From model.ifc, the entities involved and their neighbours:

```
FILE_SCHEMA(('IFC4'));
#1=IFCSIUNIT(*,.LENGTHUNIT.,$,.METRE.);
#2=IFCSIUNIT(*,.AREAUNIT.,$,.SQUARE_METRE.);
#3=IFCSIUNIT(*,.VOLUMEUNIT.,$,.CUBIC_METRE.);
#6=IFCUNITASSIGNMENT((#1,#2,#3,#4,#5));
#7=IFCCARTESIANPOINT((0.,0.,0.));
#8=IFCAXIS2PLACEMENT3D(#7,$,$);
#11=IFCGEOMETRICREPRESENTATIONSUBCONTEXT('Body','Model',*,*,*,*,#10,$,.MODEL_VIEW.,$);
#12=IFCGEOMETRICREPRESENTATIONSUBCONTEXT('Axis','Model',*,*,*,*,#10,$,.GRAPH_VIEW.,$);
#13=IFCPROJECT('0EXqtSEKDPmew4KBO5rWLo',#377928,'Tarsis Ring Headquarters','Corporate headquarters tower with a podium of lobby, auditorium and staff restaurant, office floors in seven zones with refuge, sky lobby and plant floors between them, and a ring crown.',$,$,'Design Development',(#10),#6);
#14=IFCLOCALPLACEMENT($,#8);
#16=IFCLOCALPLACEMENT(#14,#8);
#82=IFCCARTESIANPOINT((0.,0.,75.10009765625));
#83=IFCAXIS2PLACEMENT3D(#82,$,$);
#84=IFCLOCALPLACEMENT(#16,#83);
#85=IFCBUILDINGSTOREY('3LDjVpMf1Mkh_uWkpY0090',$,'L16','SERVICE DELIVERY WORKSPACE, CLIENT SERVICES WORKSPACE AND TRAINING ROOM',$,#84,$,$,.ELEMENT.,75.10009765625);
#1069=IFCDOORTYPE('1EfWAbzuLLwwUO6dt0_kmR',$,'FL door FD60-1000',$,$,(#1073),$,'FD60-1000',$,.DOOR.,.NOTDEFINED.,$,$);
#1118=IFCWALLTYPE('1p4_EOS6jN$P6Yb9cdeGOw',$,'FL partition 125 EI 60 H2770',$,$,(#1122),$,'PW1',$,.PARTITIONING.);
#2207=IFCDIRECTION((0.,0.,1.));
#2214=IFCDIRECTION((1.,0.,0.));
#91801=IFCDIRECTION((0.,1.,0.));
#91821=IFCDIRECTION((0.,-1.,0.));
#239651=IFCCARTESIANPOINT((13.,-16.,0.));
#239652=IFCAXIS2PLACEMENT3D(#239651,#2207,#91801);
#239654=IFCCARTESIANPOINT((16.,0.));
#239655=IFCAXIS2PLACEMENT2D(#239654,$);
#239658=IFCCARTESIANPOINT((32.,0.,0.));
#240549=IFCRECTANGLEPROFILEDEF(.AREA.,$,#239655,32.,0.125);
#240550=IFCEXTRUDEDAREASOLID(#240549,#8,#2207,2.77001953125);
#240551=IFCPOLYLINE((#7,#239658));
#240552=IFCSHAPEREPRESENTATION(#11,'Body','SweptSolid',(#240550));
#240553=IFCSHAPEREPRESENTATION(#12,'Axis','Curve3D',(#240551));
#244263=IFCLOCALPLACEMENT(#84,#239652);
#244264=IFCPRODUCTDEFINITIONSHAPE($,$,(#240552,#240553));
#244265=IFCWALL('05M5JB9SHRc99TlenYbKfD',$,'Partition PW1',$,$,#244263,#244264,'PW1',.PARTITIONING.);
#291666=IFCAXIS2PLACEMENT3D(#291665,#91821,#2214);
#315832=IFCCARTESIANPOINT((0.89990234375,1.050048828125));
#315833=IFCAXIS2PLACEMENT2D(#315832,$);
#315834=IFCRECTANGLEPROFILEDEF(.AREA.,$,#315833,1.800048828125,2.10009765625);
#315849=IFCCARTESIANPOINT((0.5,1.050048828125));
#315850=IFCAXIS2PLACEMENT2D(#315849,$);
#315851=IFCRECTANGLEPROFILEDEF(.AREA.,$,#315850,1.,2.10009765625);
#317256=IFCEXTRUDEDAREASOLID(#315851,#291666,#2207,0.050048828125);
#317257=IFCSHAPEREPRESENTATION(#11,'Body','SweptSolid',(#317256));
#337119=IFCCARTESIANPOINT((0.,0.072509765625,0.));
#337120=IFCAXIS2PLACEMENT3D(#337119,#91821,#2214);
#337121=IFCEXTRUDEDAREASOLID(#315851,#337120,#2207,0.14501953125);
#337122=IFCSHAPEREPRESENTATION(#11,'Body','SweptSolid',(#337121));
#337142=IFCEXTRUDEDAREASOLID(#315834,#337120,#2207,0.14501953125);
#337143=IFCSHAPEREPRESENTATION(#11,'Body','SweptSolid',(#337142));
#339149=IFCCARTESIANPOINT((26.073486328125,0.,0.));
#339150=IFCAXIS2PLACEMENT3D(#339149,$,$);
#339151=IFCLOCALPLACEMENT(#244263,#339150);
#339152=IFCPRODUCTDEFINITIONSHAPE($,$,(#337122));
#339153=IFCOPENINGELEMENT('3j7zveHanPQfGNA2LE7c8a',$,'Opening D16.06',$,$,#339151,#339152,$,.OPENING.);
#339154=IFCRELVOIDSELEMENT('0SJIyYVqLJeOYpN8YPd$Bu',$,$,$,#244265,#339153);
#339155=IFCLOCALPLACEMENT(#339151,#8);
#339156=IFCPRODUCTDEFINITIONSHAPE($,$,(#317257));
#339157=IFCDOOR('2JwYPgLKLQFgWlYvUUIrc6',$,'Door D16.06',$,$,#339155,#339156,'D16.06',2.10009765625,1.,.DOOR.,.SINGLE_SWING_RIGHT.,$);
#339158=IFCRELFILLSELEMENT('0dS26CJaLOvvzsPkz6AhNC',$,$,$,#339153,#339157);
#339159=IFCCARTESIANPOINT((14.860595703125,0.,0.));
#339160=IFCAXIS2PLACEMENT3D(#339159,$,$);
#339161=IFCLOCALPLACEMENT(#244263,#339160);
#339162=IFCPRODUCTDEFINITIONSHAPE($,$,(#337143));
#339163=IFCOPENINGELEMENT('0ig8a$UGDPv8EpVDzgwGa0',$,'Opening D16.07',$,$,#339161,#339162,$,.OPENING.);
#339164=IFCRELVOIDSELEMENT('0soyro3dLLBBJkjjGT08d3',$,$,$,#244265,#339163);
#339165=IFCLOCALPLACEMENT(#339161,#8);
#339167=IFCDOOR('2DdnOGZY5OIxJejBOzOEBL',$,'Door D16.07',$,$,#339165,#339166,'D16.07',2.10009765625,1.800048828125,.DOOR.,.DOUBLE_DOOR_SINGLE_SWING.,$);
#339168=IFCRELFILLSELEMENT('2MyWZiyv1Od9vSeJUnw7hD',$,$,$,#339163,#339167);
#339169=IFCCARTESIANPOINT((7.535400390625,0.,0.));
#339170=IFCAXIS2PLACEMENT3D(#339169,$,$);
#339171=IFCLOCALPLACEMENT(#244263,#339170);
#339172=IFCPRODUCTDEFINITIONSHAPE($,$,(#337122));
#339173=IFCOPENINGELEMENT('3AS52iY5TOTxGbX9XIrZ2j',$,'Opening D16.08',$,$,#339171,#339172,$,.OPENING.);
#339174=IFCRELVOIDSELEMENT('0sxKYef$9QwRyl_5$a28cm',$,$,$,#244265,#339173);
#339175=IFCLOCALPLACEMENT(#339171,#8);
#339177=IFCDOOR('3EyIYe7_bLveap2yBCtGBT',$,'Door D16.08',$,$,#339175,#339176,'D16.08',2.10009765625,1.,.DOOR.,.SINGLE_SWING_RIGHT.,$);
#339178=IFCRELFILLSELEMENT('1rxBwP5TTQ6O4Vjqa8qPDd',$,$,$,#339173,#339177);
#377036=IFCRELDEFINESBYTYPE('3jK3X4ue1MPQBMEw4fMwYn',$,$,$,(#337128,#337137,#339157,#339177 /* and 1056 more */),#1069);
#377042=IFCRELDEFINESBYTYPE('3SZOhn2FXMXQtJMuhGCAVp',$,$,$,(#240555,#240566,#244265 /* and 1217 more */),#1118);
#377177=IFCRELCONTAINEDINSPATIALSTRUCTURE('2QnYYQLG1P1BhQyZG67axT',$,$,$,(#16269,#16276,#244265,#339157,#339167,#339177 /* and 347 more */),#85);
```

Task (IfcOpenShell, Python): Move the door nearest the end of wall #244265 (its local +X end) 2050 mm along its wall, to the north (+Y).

```python
import ifcopenshell
import ifcopenshell.api.geometry
import ifcopenshell.util.placement
import ifcopenshell.util.unit

model = ifcopenshell.open("model.ifc")
unit_scale = ifcopenshell.util.unit.calculate_unit_scale(model)

door = model.by_guid("2JwYPgLKLQFgWlYvUUIrc6")
opening = door.FillsVoids[0].RelatingOpeningElement
wall = opening.VoidsElements[0].RelatingBuildingElement

wall_matrix = ifcopenshell.util.placement.get_local_placement(wall.ObjectPlacement)
shift = wall_matrix[:3, 0] * 2.05 / unit_scale
before = ifcopenshell.util.placement.get_local_placement(door.ObjectPlacement)[:3, 3].copy()

# The door is placed relative to its opening, so it follows when the opening moves.
matrix = ifcopenshell.util.placement.get_local_placement(opening.ObjectPlacement)
matrix[:3, 3] += shift
ifcopenshell.api.geometry.edit_object_placement(
    model, product=opening, matrix=matrix, is_si=False, should_transform_children=True
)

after = ifcopenshell.util.placement.get_local_placement(door.ObjectPlacement)[:3, 3]
print("door moved by", (after - before).round(3) + 0.0)

model.write("model_edited.ifc")
```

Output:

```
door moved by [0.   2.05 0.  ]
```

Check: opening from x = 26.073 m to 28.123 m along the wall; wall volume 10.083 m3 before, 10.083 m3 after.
